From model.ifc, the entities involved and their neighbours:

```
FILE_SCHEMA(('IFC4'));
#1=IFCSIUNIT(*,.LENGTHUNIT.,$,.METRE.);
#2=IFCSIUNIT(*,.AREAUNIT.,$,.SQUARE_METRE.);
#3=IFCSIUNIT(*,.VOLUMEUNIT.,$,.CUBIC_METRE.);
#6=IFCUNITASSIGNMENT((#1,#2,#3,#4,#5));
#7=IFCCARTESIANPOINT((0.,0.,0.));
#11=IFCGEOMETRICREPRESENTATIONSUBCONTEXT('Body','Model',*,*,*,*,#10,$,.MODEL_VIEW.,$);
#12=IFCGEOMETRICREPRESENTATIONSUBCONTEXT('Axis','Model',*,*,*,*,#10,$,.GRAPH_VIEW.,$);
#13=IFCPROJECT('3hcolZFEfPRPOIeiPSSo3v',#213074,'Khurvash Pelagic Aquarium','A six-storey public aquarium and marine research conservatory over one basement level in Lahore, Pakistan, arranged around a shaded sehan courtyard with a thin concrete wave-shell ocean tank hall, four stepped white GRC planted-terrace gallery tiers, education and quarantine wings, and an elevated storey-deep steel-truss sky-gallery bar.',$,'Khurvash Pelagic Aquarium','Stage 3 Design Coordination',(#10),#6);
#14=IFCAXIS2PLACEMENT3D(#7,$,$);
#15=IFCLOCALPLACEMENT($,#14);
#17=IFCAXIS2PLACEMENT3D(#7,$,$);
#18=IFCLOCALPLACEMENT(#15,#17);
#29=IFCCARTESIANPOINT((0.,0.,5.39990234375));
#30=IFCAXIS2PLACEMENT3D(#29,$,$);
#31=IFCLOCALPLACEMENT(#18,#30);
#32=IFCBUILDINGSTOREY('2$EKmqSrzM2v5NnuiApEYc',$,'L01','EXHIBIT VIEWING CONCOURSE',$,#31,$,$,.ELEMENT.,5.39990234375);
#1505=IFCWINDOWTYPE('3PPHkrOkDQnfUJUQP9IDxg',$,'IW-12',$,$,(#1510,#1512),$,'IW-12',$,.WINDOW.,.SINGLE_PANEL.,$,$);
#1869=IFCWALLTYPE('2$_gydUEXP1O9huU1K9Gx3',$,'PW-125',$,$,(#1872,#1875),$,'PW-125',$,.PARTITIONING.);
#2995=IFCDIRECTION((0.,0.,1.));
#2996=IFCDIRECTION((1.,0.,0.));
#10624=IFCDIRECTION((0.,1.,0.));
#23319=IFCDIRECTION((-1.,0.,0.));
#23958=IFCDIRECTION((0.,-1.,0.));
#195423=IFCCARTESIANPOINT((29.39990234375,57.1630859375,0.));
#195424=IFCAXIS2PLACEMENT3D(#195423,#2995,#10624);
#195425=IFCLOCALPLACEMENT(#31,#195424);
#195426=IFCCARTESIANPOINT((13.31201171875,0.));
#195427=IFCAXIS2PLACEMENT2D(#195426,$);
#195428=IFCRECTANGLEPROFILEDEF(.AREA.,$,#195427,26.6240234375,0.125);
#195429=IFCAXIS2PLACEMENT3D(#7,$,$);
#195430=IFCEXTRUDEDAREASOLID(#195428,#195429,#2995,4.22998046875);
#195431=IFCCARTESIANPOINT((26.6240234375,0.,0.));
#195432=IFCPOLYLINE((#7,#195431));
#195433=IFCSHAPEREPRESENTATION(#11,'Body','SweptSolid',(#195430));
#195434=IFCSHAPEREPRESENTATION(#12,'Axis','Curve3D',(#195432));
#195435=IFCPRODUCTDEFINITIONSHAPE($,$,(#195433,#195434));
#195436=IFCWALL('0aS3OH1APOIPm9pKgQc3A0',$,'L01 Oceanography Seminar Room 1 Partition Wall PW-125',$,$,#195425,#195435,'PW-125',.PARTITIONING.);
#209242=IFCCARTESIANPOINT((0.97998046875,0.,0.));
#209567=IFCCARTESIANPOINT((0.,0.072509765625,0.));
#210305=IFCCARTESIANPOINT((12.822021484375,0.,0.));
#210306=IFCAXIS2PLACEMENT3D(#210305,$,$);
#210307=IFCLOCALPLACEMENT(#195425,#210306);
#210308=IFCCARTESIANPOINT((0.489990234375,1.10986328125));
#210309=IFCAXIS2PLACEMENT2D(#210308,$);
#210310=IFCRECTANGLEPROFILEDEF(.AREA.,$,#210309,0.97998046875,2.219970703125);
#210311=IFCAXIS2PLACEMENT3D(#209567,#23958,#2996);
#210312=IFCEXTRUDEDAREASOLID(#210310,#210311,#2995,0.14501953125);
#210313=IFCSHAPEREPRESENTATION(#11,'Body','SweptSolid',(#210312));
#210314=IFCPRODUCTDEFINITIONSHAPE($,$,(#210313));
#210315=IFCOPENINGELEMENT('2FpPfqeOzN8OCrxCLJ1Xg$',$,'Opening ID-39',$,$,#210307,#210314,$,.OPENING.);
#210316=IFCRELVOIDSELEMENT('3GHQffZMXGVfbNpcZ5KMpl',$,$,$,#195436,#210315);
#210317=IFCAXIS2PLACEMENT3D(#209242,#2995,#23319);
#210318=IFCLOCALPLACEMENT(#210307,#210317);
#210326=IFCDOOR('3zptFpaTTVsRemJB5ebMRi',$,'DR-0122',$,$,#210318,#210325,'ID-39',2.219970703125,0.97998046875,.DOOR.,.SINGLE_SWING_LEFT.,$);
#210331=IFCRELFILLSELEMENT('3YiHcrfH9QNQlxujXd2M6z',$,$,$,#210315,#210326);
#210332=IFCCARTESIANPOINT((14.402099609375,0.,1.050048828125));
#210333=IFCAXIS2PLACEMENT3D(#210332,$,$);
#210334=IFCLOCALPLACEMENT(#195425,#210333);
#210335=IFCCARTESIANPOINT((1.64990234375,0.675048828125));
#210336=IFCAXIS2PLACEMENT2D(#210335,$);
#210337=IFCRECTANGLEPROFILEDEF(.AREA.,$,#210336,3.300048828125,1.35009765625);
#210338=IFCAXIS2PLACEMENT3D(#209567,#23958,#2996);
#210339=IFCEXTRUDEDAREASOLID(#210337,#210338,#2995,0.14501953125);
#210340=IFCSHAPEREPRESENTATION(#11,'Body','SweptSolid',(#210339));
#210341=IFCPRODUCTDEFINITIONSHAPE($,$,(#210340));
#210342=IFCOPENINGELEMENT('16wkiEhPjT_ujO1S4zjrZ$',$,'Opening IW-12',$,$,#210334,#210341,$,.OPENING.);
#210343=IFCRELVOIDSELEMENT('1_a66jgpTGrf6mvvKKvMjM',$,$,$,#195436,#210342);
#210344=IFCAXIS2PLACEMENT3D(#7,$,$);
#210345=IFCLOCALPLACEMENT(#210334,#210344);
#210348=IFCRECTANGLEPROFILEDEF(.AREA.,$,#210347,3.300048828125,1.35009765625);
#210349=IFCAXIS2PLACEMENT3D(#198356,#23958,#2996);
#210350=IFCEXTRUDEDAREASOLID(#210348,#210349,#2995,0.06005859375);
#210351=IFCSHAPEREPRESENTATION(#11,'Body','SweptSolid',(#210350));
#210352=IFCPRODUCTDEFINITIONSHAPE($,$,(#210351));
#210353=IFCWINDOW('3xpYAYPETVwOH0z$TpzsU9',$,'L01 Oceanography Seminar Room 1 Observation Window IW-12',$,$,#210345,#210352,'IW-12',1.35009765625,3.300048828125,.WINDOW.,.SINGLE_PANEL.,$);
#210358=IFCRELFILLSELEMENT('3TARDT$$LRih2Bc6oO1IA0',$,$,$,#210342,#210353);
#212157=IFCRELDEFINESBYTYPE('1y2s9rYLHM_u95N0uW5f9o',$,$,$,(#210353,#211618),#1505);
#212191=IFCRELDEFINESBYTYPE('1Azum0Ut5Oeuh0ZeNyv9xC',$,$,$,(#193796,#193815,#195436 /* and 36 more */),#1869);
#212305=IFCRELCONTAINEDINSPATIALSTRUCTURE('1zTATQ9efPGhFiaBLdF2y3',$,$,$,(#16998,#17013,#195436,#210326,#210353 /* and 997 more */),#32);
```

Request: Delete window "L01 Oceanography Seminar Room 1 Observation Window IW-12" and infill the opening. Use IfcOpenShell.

```python
import ifcopenshell
import ifcopenshell.api.feature
import ifcopenshell.api.root
import ifcopenshell.geom
import ifcopenshell.util.shape

model = ifcopenshell.open("model.ifc")
settings = ifcopenshell.geom.settings()


def volume(element):
    """Net volume in cubic metres, openings subtracted."""
    shape = ifcopenshell.geom.create_shape(settings, element)
    return ifcopenshell.util.shape.get_volume(shape.geometry)


window = model.by_guid("3xpYAYPETVwOH0z$TpzsU9")
opening = window.FillsVoids[0].RelatingOpeningElement
wall = opening.VoidsElements[0].RelatingBuildingElement
before = volume(wall)

ifcopenshell.api.root.remove_product(model, product=window)
ifcopenshell.api.feature.remove_feature(model, feature=opening)

after = volume(wall)

print(f"wall volume {before:.3f} -> {after:.3f} m3")

model.write("model_rev.ifc")
```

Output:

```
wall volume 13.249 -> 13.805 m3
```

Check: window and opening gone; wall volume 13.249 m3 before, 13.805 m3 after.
